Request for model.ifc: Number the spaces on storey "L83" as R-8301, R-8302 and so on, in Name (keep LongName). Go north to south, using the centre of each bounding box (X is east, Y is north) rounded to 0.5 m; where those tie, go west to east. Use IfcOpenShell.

First a look at what the model holds.

```python
import ifcopenshell
import ifcopenshell.util.element
import ifcopenshell.util.placement

model = ifcopenshell.open("model.ifc")
print(model.schema)
storey = next(s for s in model.by_type("IfcBuildingStorey") if s.Name == "L83")
spaces = [e for e in ifcopenshell.util.element.get_decomposition(storey) if e.is_a("IfcSpace")]
for e in sorted(spaces, key=lambda e: e.id()):
    origin = ifcopenshell.util.placement.get_local_placement(e.ObjectPlacement)[:3, 3]
    print(e.id(), e.Name, e.LongName, origin.round(2) + 0.0, sep=" | ")
```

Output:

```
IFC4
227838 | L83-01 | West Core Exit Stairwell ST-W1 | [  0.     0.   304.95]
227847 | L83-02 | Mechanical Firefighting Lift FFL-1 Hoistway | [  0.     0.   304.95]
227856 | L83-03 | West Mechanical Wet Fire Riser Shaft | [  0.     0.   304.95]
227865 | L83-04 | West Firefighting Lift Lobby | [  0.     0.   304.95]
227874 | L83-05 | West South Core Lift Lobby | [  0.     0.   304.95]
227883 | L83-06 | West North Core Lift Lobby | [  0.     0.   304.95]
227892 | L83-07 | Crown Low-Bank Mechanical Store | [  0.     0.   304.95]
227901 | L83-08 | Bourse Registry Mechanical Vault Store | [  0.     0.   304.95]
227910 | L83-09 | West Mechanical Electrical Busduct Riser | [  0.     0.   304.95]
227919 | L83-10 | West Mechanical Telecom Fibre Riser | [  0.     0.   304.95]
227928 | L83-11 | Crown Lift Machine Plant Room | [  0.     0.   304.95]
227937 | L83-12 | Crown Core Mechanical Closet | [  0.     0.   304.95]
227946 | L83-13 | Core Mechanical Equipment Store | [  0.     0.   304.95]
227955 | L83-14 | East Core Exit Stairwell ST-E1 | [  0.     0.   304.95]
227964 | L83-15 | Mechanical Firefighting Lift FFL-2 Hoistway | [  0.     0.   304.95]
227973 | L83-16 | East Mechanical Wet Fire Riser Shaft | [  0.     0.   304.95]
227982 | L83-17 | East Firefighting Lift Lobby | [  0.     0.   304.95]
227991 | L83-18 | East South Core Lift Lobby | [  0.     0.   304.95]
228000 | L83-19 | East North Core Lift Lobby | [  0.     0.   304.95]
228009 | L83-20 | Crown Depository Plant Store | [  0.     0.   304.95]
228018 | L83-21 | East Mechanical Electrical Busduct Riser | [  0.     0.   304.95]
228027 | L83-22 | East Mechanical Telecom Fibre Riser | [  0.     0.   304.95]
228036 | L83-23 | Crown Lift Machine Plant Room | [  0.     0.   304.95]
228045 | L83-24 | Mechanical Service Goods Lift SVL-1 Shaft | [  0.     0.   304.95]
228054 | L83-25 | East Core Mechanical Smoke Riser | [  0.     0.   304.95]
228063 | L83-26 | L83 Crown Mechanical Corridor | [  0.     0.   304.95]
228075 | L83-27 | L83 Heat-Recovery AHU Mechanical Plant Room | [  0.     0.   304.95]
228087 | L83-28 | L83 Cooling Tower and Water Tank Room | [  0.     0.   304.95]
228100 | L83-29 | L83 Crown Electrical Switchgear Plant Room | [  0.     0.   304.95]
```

```python
import ifcopenshell
import ifcopenshell.geom
import ifcopenshell.util.element
import ifcopenshell.util.shape

model = ifcopenshell.open("model.ifc")
settings = ifcopenshell.geom.settings()
settings.set("use-world-coords", True)


def centre(element):
    shape = ifcopenshell.geom.create_shape(settings, element)
    return ifcopenshell.util.shape.get_bbox_centroid(shape.geometry)


storey = next(s for s in model.by_type("IfcBuildingStorey") if s.Name == "L83")
spaces = [e for e in ifcopenshell.util.element.get_decomposition(storey) if e.is_a("IfcSpace")]

# Insertion points can sit at a corner or the storey origin, so sort by the geometry (in metres).
centres = {e: centre(e) for e in spaces}
spaces.sort(key=lambda e: (-round(centres[e][1] / 0.5), centres[e][0]))

for i, e in enumerate(spaces, start=1):
    number = f"R-83{i:02d}"
    e.Name = number
    print(e.id(), number)

model.write("model_edited.ifc")
```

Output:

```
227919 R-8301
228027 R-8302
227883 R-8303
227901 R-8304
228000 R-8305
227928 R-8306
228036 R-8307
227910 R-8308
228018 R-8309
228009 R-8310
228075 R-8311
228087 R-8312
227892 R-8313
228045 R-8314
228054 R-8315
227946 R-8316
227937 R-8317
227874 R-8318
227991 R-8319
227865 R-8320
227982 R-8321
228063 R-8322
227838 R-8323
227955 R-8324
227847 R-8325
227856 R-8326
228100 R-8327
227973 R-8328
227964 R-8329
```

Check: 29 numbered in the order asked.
